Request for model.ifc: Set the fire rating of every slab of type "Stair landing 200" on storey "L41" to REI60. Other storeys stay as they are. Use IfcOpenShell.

First a look at what the model holds.

```python
import ifcopenshell
import ifcopenshell.util.element

model = ifcopenshell.open("model.ifc")
print(model.schema)
storey = next(s for s in model.by_type("IfcBuildingStorey") if s.Name == "L41")
slabs = [e for e in ifcopenshell.util.element.get_decomposition(storey) if e.is_a("IfcSlab")]
seen = {}
for e in slabs:
    element_type = ifcopenshell.util.element.get_type(e)
    key = (element_type.Name if element_type != e and element_type else None, ifcopenshell.util.element.get_pset(e, "Pset_SlabCommon", "FireRating"))
    seen[key] = seen.get(key, 0) + 1
for (name, value), count in sorted(seen.items(), key=str):
    print(count, "x", name, "|", value)
```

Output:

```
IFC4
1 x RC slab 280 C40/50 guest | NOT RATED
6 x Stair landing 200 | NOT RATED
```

```python
import ifcopenshell
import ifcopenshell.api.pset
import ifcopenshell.util.element

model = ifcopenshell.open("model.ifc")

storey = next(s for s in model.by_type("IfcBuildingStorey") if s.Name == "L41")
slabs = [e for e in ifcopenshell.util.element.get_decomposition(storey) if e.is_a("IfcSlab")]

count = 0
for e in slabs:
    element_type = ifcopenshell.util.element.get_type(e)
    if element_type in (None, e) or element_type.Name != "Stair landing 200":
        continue
    # add_pset returns the element's existing set when there is one.
    pset = ifcopenshell.api.pset.add_pset(model, product=e, name="Pset_SlabCommon")
    ifcopenshell.api.pset.edit_pset(model, pset=pset, properties={"FireRating": "REI60"})
    count += 1

print(count, "slabs updated")

model.write("model_updated.ifc")
```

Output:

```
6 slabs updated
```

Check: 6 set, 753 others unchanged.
